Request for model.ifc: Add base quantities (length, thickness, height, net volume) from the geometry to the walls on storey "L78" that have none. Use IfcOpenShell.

First a look at what the model holds.

```python
import ifcopenshell
import ifcopenshell.util.element
import ifcopenshell.util.unit

model = ifcopenshell.open("model.ifc")
print(model.schema)
for unit_type in ("LENGTHUNIT", "AREAUNIT", "VOLUMEUNIT"):
    print(unit_type, ifcopenshell.util.unit.calculate_unit_scale(model, unit_type))
storey = next(s for s in model.by_type("IfcBuildingStorey") if s.Name == "L78")
walls = [e for e in ifcopenshell.util.element.get_decomposition(storey) if e.is_a("IfcWall")]
for e in sorted(walls, key=lambda e: e.id()):
    print(e.id(), e.is_a(), e.Name, list(ifcopenshell.util.element.get_psets(e, qtos_only=True)), sep=" | ")
```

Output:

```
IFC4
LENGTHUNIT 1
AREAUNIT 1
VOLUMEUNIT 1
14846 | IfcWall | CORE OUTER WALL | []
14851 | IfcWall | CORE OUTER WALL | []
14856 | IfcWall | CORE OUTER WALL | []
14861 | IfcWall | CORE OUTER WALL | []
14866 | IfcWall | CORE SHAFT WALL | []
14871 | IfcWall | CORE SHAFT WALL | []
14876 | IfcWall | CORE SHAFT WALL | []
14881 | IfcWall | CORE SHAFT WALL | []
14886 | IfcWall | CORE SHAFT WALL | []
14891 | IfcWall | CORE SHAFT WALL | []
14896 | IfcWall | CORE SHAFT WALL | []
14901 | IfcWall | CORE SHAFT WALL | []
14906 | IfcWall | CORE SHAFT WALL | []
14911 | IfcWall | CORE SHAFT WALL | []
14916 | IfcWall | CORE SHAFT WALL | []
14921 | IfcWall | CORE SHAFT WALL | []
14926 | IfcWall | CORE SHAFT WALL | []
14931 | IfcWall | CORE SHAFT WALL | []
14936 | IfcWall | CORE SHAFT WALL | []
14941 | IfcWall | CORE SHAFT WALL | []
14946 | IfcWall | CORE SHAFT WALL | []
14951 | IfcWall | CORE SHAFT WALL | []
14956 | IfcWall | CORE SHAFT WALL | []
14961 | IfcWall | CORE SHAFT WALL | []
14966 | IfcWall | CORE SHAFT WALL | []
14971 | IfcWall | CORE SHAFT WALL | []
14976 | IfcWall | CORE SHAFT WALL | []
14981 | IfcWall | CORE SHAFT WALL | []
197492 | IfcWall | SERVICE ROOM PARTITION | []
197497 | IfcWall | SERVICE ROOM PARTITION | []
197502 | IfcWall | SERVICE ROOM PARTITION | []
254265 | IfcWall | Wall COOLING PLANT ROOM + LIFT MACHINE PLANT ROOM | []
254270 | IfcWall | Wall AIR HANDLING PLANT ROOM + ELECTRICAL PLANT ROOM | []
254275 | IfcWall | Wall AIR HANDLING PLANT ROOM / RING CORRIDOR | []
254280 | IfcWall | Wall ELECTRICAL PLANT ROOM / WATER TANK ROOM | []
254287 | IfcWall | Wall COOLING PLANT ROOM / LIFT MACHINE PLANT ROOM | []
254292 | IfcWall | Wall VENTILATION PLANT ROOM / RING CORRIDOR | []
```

```python
import ifcopenshell
import ifcopenshell.api.pset
import ifcopenshell.geom
import ifcopenshell.util.element
import ifcopenshell.util.shape
import ifcopenshell.util.unit

model = ifcopenshell.open("model.ifc")
unit_scale = ifcopenshell.util.unit.calculate_unit_scale(model)
volume_scale = ifcopenshell.util.unit.calculate_unit_scale(model, "VOLUMEUNIT")
settings = ifcopenshell.geom.settings()

storey = next(s for s in model.by_type("IfcBuildingStorey") if s.Name == "L78")
walls = [e for e in ifcopenshell.util.element.get_decomposition(storey) if e.is_a("IfcWall")]

for e in sorted(walls, key=lambda e: e.id()):
    if ifcopenshell.util.element.get_psets(e, qtos_only=True, should_inherit=False):
        continue
    # Geometry comes back in metres, in the element's own axes.
    shape = ifcopenshell.geom.create_shape(settings, e)
    values = {
        "Length": ifcopenshell.util.shape.get_x(shape.geometry) / unit_scale,
        "Width": ifcopenshell.util.shape.get_y(shape.geometry) / unit_scale,
        "Height": ifcopenshell.util.shape.get_z(shape.geometry) / unit_scale,
        "NetVolume": ifcopenshell.util.shape.get_volume(shape.geometry) / volume_scale,
    }
    qto = ifcopenshell.api.pset.add_qto(model, product=e, name="Qto_WallBaseQuantities")
    ifcopenshell.api.pset.edit_qto(model, qto=qto, properties=values)
    print(e.id(), {k: round(v, 3) for k, v in values.items()})

model.write("model_edited.ifc")
```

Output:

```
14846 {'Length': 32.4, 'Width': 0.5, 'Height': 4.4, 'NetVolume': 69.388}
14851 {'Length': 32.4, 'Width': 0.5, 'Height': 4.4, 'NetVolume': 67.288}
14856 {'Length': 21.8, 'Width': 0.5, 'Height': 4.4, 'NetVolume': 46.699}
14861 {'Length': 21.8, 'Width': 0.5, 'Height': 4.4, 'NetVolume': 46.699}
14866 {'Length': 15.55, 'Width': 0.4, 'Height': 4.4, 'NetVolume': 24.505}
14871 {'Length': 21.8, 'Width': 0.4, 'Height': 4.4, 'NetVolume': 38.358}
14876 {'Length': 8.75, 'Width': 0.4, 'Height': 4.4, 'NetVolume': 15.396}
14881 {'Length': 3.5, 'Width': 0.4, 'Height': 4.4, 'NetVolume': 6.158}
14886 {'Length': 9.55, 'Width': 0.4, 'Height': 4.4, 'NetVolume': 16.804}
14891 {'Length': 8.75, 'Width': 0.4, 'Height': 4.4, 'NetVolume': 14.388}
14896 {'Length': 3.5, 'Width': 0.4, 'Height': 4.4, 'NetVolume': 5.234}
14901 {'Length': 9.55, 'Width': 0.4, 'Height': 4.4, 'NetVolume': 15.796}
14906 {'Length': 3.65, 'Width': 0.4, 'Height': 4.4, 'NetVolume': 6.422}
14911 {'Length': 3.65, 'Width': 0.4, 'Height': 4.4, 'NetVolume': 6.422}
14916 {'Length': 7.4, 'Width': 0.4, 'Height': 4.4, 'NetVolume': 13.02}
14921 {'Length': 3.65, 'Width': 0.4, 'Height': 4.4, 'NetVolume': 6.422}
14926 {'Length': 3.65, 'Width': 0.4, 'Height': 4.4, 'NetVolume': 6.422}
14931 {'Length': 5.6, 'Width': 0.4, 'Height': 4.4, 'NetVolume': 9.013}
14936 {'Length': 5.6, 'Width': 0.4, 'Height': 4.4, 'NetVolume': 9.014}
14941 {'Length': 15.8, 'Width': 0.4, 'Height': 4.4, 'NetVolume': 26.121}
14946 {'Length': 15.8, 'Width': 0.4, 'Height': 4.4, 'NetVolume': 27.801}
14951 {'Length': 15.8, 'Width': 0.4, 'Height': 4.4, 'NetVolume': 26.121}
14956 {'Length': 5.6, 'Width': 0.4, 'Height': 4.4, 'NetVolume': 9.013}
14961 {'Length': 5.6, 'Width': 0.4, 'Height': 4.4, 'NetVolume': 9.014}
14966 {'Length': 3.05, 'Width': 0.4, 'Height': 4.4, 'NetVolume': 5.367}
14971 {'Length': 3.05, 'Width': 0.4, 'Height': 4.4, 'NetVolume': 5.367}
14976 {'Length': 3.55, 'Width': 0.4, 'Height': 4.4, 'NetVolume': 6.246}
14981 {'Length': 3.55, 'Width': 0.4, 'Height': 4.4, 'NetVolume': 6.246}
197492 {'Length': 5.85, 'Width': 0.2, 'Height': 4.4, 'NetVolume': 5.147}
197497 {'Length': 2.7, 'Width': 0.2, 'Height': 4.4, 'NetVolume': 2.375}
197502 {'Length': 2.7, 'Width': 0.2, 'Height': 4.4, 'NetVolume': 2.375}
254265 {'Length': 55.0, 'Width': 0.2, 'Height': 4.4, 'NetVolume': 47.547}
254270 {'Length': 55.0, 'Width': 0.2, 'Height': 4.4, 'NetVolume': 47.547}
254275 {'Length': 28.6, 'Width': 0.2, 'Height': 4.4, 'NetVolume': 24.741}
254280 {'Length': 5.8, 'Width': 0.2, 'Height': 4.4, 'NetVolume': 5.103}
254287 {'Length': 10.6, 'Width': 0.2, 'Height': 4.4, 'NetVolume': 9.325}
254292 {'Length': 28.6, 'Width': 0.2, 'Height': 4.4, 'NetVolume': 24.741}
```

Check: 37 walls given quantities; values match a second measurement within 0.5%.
